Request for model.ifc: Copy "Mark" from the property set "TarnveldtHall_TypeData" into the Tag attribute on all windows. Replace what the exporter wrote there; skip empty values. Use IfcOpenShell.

First a look at what the model holds.

```python
import ifcopenshell
import ifcopenshell.util.element

model = ifcopenshell.open("model.ifc")
print(model.schema)
windows = model.by_type("IfcWindow")
print(len(windows), "windows")
for e in windows[:8]:
    source = ifcopenshell.util.element.get_pset(e, "TarnveldtHall_TypeData", "Mark")
    target = e.Tag
    print(e.id(), repr(source), repr(target), sep=" | ")
```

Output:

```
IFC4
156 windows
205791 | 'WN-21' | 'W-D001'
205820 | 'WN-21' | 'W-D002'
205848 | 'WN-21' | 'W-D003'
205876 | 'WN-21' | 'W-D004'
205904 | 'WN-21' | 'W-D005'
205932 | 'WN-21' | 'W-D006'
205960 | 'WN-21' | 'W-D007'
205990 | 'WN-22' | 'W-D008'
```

```python
import ifcopenshell
import ifcopenshell.util.element

model = ifcopenshell.open("model.ifc")

count = 0
for e in model.by_type("IfcWindow"):
    value = ifcopenshell.util.element.get_pset(e, "TarnveldtHall_TypeData", "Mark")
    current = e.Tag
    if not value or not value.strip() or current == value:
        continue
    e.Tag = value
    count += 1

print(count, "windows updated")

model.write("model_updated.ifc")
```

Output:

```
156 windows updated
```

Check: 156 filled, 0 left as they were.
